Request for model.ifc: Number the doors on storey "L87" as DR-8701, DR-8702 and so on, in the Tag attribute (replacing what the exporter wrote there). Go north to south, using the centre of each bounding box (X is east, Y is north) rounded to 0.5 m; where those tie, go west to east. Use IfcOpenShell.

First a look at what the model holds.

```python
import ifcopenshell
import ifcopenshell.util.element
import ifcopenshell.util.placement

model = ifcopenshell.open("model.ifc")
print(model.schema)
storey = next(s for s in model.by_type("IfcBuildingStorey") if s.Name == "L87")
doors = [e for e in ifcopenshell.util.element.get_decomposition(storey) if e.is_a("IfcDoor")]
for e in sorted(doors, key=lambda e: e.id()):
    origin = ifcopenshell.util.placement.get_local_placement(e.ObjectPlacement)[:3, 3]
    print(e.id(), e.Tag, e.Name, origin.round(2) + 0.0, sep=" | ")
```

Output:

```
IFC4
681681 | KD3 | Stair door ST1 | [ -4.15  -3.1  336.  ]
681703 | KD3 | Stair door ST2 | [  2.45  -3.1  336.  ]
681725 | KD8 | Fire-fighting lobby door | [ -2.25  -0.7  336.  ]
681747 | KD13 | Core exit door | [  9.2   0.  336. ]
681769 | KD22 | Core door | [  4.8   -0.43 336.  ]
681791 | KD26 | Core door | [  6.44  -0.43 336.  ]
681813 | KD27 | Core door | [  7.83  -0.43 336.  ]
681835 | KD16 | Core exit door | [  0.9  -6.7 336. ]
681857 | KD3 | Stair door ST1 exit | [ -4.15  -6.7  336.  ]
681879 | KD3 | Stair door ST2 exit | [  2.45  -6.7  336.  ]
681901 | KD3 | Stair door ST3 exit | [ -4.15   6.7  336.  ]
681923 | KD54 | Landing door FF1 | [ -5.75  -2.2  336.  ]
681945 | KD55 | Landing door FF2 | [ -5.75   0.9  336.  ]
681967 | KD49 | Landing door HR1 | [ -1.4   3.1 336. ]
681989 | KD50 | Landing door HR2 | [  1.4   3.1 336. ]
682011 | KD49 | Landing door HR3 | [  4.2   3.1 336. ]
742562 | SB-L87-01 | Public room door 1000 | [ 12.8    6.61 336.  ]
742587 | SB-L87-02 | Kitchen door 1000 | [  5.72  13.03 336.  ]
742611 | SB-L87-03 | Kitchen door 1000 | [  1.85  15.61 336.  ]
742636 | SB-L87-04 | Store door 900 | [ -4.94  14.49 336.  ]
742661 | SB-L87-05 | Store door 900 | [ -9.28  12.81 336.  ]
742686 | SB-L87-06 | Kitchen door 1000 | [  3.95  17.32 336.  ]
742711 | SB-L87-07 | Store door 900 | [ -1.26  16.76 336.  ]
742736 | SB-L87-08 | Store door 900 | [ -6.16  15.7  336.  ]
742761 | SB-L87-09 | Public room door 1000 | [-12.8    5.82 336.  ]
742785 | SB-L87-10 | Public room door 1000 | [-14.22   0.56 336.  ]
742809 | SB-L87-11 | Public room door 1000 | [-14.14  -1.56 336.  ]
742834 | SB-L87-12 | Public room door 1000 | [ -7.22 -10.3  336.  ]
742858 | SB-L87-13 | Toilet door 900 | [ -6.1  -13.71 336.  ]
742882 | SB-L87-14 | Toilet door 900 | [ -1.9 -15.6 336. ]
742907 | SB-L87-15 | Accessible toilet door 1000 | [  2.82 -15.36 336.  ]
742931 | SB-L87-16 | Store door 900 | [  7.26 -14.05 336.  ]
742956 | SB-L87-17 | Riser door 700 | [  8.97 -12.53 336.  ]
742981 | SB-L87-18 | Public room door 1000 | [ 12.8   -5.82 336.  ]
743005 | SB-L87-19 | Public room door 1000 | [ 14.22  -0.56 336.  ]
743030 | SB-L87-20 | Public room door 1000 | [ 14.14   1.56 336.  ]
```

```python
import ifcopenshell
import ifcopenshell.geom
import ifcopenshell.util.element
import ifcopenshell.util.shape

model = ifcopenshell.open("model.ifc")
settings = ifcopenshell.geom.settings()
settings.set("use-world-coords", True)


def centre(element):
    shape = ifcopenshell.geom.create_shape(settings, element)
    return ifcopenshell.util.shape.get_bbox_centroid(shape.geometry)


storey = next(s for s in model.by_type("IfcBuildingStorey") if s.Name == "L87")
doors = [e for e in ifcopenshell.util.element.get_decomposition(storey) if e.is_a("IfcDoor")]

# Insertion points can sit at a corner or the storey origin, so sort by the geometry (in metres).
centres = {e: centre(e) for e in doors}
doors.sort(key=lambda e: (-round(centres[e][1] / 0.5), centres[e][0]))

for i, e in enumerate(doors, start=1):
    number = f"DR-87{i:02d}"
    e.Tag = number
    print(e.id(), number)

model.write("model_v2.ifc")
```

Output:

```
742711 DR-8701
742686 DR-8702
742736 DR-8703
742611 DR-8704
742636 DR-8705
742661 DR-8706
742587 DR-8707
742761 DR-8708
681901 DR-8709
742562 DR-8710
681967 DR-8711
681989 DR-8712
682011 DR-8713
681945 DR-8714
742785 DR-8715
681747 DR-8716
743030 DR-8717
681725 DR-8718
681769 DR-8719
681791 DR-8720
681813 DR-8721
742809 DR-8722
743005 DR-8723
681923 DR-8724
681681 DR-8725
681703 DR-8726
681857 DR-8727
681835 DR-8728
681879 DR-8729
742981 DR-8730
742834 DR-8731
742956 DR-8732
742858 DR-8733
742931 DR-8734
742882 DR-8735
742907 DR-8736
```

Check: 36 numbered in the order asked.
